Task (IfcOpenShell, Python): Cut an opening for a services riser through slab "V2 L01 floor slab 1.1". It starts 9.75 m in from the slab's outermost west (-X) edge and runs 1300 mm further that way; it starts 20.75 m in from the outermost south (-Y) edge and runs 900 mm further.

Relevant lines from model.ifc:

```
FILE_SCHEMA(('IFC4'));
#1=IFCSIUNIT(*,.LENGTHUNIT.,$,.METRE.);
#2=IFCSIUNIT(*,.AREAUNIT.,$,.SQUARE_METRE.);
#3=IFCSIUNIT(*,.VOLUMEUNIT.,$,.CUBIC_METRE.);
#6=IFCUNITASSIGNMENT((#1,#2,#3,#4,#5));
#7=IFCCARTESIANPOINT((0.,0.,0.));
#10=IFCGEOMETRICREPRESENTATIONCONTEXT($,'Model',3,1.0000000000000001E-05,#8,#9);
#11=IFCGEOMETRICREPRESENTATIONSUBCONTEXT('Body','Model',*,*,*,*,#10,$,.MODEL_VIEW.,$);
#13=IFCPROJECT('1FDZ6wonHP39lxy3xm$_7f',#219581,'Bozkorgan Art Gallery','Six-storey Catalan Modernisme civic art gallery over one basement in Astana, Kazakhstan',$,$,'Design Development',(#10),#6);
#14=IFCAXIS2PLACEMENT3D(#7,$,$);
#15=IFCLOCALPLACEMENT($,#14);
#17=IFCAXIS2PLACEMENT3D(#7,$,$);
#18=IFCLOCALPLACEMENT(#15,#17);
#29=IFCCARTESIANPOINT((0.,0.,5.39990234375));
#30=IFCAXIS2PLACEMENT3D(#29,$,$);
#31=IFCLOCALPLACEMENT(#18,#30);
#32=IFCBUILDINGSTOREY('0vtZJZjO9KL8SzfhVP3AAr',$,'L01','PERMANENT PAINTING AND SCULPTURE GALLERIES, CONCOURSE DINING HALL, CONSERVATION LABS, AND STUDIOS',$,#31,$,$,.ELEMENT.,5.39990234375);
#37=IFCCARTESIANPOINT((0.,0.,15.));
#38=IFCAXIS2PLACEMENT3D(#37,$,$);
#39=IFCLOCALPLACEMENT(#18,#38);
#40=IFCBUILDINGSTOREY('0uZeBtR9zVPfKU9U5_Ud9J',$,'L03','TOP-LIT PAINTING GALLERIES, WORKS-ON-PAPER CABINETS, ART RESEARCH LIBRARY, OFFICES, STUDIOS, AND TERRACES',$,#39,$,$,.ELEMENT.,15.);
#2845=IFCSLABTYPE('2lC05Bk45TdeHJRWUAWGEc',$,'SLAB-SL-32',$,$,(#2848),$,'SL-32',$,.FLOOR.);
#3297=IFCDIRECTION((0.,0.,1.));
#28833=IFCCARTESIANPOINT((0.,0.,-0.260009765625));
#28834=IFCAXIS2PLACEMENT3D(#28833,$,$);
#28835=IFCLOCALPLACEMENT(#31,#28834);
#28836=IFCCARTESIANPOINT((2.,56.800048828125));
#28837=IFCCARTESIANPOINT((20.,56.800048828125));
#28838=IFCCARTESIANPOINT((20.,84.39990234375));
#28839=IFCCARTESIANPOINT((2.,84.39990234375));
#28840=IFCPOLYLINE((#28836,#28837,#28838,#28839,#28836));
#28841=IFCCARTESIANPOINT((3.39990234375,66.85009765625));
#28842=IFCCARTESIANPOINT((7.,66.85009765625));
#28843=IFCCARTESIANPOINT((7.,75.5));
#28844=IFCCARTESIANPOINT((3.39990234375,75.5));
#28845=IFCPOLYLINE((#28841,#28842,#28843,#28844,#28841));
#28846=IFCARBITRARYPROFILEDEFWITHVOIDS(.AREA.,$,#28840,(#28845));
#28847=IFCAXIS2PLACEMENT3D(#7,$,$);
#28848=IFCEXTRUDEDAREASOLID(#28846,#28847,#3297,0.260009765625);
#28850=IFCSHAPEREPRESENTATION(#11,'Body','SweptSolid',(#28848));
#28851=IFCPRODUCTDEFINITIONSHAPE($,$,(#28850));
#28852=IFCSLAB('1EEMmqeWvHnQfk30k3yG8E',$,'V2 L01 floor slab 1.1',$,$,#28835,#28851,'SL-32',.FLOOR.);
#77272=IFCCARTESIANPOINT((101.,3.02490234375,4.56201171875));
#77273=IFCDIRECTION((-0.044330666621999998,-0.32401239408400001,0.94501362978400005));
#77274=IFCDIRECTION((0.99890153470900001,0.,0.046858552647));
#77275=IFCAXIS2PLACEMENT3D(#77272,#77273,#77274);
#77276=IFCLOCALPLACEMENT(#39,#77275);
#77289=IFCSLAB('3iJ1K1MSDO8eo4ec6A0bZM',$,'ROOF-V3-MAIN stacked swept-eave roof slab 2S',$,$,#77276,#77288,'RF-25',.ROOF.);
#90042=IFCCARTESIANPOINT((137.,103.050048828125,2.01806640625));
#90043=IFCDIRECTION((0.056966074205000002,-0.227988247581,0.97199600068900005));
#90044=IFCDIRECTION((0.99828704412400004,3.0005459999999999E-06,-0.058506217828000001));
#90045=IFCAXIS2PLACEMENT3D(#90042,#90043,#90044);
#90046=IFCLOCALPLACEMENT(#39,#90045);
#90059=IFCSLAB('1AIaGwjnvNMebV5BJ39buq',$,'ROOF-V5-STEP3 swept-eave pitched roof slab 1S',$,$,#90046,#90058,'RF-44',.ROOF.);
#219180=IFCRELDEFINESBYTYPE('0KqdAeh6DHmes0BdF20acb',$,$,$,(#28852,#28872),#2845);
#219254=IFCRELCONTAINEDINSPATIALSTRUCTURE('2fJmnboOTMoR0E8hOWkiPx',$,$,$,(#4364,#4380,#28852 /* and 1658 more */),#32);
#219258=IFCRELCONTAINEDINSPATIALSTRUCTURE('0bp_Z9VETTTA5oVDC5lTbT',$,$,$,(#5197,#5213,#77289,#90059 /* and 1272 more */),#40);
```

```python
import numpy as np
import ifcopenshell
import ifcopenshell.api.feature
import ifcopenshell.api.geometry
import ifcopenshell.api.root
import ifcopenshell.geom
import ifcopenshell.util.placement
import ifcopenshell.util.representation
import ifcopenshell.util.shape
import ifcopenshell.util.unit

model = ifcopenshell.open("model.ifc")
unit_scale = ifcopenshell.util.unit.calculate_unit_scale(model)
settings = ifcopenshell.geom.settings()


def volume(element):
    """Net volume in cubic metres, openings subtracted."""
    shape = ifcopenshell.geom.create_shape(settings, element)
    return ifcopenshell.util.shape.get_volume(shape.geometry)


slab = model.by_id(28852)
before = volume(slab)

# Extent in the slab's own axes, in metres. The edges named are its -X and -Y sides.
slab_shape = ifcopenshell.geom.create_shape(settings, slab)
vertices = ifcopenshell.util.shape.get_vertices(slab_shape.geometry)
x_min, y_min, bottom = vertices.min(axis=0)
top = vertices[:, 2].max()

opening = ifcopenshell.api.root.create_entity(model, ifc_class="IfcOpeningElement", name="Services riser opening", predefined_type="OPENING")
context = ifcopenshell.util.representation.get_context(model, "Model", "Body", "MODEL_VIEW")
width, depth = 1.3, 0.9
outline = [(0.0, 0.0), (width, 0.0), (width, depth), (0.0, depth), (0.0, 0.0)]
# Overshoot both faces by 50 mm so the cut is clean.
shape = ifcopenshell.api.geometry.add_slab_representation(
    model, context=context, depth=top - bottom + 0.1, polyline=outline
)
ifcopenshell.api.geometry.assign_representation(model, product=opening, representation=shape)

matrix = ifcopenshell.util.placement.get_local_placement(slab.ObjectPlacement)
matrix[:, 3] = matrix @ np.append(np.array([x_min + 9.75, y_min + 20.75, bottom - 0.05]) / unit_scale, 1.0)
ifcopenshell.api.geometry.edit_object_placement(model, product=opening, matrix=matrix, is_si=False)
ifcopenshell.api.feature.add_feature(model, feature=opening, element=slab)

after = volume(slab)

print(f"slab volume {before:.3f} -> {after:.3f} m3")

model.write("model_v2.ifc")
```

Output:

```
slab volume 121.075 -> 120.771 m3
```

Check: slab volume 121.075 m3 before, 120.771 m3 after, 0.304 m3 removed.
